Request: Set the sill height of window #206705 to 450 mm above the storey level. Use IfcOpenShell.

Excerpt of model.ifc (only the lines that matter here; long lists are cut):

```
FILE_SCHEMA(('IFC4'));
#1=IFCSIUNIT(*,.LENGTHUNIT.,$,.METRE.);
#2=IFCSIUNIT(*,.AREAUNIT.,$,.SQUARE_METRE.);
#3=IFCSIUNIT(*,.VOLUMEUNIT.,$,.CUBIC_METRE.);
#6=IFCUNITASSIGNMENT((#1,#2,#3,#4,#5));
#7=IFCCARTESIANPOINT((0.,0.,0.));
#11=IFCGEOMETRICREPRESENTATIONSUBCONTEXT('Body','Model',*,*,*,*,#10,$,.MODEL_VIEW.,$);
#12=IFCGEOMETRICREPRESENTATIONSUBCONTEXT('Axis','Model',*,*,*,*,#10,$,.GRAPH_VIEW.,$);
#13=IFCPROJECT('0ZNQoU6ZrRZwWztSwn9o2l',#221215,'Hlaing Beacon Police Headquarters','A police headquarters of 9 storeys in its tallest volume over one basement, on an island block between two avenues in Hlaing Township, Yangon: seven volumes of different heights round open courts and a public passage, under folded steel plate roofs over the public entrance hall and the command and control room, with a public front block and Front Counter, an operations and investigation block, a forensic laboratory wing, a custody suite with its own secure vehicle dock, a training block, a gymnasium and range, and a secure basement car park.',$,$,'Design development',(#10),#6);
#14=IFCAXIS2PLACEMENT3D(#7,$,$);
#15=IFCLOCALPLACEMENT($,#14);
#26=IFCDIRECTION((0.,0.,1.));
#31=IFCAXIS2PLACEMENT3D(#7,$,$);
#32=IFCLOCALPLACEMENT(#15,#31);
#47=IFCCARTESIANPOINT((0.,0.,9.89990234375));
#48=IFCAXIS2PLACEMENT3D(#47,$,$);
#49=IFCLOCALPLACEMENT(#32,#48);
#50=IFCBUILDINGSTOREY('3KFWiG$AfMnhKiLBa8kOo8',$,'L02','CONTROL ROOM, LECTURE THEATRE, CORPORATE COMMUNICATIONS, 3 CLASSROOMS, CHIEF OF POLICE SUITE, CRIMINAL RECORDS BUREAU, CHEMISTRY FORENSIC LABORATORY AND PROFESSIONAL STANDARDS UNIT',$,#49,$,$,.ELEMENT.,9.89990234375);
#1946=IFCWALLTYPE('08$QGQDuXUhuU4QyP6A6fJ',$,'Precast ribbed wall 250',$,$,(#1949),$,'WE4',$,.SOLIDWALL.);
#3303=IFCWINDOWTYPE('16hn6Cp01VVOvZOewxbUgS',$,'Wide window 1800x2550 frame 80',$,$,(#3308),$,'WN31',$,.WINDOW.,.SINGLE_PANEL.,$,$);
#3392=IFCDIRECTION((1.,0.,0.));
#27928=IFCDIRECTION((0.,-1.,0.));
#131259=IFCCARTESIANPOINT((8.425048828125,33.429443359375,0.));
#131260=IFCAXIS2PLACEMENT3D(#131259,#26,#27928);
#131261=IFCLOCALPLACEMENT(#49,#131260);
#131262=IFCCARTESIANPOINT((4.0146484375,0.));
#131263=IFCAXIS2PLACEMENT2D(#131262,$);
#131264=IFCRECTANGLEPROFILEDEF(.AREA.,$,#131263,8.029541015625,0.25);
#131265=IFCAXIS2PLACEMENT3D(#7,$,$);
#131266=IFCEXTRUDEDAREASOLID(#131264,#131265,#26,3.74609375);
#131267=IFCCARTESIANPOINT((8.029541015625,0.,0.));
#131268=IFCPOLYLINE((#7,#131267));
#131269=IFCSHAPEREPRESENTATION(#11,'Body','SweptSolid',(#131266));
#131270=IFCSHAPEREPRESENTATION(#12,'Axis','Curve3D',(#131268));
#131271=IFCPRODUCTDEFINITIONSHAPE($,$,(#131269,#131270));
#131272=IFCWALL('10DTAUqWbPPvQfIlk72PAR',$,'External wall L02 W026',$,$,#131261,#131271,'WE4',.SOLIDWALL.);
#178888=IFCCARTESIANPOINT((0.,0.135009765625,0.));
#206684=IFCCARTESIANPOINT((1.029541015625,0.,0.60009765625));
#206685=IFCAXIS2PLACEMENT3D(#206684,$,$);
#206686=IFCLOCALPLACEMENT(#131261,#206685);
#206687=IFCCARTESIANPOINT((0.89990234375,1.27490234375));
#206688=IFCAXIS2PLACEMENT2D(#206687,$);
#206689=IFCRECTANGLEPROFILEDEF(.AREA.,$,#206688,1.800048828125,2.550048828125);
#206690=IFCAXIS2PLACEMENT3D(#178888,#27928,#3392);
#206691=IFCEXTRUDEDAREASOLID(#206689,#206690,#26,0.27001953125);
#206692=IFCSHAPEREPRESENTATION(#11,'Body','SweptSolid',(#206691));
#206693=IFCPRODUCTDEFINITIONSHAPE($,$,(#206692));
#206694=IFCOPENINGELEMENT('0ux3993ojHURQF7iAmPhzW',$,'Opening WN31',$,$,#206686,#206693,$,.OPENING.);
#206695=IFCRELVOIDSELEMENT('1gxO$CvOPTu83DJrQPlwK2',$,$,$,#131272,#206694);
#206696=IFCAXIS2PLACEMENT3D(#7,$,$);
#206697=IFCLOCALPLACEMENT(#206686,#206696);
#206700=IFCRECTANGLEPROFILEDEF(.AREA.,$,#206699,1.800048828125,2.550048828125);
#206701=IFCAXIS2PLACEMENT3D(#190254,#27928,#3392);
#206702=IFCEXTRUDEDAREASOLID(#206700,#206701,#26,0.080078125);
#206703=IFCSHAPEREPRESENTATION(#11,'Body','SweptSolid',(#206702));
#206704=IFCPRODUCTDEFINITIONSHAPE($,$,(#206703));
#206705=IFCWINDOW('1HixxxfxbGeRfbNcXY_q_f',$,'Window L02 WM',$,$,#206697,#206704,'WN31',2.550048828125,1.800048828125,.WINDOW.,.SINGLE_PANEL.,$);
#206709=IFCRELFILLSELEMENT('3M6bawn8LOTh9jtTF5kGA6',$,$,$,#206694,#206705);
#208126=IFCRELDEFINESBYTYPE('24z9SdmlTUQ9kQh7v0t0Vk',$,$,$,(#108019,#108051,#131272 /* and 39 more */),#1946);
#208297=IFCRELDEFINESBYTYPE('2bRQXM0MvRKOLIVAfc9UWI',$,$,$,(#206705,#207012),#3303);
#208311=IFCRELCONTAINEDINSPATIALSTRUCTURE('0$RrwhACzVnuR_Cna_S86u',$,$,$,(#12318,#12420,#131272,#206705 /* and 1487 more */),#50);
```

```python
import numpy as np
import ifcopenshell
import ifcopenshell.api.geometry
import ifcopenshell.geom
import ifcopenshell.util.element
import ifcopenshell.util.placement
import ifcopenshell.util.shape
import ifcopenshell.util.unit

model = ifcopenshell.open("model.ifc")
unit_scale = ifcopenshell.util.unit.calculate_unit_scale(model)

window = model.by_guid("1HixxxfxbGeRfbNcXY_q_f")
opening = window.FillsVoids[0].RelatingOpeningElement
storey = ifcopenshell.util.element.get_container(window, ifc_class="IfcBuildingStorey")
level = ifcopenshell.util.placement.get_local_placement(storey.ObjectPlacement)[2, 3]

# The opening's origin need not be at the sill, so measure its lowest point.
shape = ifcopenshell.geom.create_shape(ifcopenshell.geom.settings(), opening)
bottom = ifcopenshell.util.shape.get_shape_bottom_elevation(shape, shape.geometry) / unit_scale
dz = level + 0.45 / unit_scale - bottom

shift = np.array([0.0, 0.0, dz])
# The window is placed relative to its opening, so it follows when the opening moves.
matrix = ifcopenshell.util.placement.get_local_placement(opening.ObjectPlacement)
matrix[:3, 3] += shift
ifcopenshell.api.geometry.edit_object_placement(
    model, product=opening, matrix=matrix, is_si=False, should_transform_children=True
)

print(f"moved by {dz * unit_scale:+.3f} m")

model.write("model-out.ifc")
```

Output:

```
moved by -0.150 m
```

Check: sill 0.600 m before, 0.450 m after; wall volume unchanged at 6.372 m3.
